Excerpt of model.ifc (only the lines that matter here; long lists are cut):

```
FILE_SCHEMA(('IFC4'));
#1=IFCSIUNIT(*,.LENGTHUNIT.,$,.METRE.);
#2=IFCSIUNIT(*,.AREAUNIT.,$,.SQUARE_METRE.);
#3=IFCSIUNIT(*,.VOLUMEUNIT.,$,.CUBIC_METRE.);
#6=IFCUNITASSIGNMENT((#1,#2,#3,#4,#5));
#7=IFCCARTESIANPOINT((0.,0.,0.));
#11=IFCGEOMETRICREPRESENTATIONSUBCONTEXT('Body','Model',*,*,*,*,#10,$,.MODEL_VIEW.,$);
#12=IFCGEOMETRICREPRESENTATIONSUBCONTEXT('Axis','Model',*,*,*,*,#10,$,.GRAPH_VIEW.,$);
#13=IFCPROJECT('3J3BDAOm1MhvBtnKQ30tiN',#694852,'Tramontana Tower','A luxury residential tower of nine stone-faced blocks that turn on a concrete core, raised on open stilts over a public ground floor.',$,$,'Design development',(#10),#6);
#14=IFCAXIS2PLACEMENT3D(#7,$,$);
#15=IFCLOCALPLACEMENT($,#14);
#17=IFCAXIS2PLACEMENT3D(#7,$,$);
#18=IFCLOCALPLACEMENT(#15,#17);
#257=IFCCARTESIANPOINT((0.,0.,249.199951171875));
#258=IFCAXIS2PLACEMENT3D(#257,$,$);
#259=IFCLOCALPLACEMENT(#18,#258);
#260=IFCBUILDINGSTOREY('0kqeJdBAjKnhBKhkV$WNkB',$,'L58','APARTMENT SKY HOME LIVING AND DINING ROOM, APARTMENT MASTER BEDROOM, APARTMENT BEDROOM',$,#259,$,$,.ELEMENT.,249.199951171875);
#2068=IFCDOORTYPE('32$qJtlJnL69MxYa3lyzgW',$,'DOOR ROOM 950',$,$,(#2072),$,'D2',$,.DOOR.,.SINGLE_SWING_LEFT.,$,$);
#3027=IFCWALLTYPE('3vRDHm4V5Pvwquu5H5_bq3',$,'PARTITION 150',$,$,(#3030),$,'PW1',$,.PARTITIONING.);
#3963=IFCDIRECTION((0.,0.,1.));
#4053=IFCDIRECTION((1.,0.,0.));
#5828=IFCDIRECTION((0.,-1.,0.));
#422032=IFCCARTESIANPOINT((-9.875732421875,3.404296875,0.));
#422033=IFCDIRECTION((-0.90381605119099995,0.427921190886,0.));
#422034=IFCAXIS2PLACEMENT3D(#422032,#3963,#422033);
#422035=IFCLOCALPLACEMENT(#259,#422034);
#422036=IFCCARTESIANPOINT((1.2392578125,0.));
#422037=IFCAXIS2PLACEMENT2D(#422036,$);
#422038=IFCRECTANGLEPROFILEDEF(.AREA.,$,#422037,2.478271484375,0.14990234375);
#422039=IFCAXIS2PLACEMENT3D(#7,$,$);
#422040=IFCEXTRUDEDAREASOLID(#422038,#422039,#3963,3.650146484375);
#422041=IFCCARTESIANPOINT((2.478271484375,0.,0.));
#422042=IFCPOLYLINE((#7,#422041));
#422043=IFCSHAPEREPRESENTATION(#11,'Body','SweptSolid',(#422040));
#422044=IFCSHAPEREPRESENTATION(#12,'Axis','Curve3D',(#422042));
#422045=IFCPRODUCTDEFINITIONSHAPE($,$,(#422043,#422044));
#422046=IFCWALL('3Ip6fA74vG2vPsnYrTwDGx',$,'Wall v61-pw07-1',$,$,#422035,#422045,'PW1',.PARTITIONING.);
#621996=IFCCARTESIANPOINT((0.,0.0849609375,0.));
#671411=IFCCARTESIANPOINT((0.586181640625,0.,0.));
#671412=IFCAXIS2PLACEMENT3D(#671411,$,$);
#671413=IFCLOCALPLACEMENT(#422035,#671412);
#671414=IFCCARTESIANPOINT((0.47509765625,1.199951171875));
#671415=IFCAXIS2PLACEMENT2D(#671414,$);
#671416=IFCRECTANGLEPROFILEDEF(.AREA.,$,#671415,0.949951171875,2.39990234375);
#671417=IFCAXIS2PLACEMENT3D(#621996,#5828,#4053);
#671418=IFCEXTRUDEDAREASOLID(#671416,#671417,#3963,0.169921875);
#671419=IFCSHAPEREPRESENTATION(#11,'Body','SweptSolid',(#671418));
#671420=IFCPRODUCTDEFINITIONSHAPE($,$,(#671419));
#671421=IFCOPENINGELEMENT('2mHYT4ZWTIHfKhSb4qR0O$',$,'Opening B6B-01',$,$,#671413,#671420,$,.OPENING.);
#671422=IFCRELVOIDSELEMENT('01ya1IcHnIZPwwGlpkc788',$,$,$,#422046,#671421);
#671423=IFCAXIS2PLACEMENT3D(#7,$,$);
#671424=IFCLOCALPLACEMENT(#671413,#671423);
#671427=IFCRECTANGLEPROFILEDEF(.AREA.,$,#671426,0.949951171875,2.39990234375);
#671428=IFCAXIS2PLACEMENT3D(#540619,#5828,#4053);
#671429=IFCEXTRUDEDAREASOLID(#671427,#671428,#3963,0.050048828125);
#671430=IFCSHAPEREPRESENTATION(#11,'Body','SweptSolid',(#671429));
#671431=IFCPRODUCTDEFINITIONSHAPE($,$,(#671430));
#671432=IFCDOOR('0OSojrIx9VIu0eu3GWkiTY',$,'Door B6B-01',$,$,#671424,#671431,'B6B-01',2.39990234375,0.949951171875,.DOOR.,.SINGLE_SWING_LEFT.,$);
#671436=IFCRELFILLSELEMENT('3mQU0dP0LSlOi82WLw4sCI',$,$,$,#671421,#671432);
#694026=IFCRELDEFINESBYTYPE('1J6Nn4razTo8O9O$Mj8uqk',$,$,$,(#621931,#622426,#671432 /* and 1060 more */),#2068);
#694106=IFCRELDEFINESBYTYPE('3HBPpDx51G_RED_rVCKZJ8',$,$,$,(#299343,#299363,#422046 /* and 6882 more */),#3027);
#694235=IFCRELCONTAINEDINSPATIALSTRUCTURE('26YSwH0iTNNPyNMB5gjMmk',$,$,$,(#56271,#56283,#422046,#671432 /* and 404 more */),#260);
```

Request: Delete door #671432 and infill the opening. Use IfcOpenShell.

```python
import ifcopenshell
import ifcopenshell.api.feature
import ifcopenshell.api.root
import ifcopenshell.geom
import ifcopenshell.util.shape

model = ifcopenshell.open("model.ifc")
settings = ifcopenshell.geom.settings()


def volume(element):
    """Net volume in cubic metres, openings subtracted."""
    shape = ifcopenshell.geom.create_shape(settings, element)
    return ifcopenshell.util.shape.get_volume(shape.geometry)


door = model.by_id(671432)
opening = door.FillsVoids[0].RelatingOpeningElement
wall = opening.VoidsElements[0].RelatingBuildingElement
before = volume(wall)

ifcopenshell.api.root.remove_product(model, product=door)
ifcopenshell.api.feature.remove_feature(model, feature=opening)

after = volume(wall)

print(f"wall volume {before:.3f} -> {after:.3f} m3")

model.write("model_updated.ifc")
```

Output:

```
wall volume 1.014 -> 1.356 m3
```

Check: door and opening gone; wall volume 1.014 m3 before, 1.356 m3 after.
